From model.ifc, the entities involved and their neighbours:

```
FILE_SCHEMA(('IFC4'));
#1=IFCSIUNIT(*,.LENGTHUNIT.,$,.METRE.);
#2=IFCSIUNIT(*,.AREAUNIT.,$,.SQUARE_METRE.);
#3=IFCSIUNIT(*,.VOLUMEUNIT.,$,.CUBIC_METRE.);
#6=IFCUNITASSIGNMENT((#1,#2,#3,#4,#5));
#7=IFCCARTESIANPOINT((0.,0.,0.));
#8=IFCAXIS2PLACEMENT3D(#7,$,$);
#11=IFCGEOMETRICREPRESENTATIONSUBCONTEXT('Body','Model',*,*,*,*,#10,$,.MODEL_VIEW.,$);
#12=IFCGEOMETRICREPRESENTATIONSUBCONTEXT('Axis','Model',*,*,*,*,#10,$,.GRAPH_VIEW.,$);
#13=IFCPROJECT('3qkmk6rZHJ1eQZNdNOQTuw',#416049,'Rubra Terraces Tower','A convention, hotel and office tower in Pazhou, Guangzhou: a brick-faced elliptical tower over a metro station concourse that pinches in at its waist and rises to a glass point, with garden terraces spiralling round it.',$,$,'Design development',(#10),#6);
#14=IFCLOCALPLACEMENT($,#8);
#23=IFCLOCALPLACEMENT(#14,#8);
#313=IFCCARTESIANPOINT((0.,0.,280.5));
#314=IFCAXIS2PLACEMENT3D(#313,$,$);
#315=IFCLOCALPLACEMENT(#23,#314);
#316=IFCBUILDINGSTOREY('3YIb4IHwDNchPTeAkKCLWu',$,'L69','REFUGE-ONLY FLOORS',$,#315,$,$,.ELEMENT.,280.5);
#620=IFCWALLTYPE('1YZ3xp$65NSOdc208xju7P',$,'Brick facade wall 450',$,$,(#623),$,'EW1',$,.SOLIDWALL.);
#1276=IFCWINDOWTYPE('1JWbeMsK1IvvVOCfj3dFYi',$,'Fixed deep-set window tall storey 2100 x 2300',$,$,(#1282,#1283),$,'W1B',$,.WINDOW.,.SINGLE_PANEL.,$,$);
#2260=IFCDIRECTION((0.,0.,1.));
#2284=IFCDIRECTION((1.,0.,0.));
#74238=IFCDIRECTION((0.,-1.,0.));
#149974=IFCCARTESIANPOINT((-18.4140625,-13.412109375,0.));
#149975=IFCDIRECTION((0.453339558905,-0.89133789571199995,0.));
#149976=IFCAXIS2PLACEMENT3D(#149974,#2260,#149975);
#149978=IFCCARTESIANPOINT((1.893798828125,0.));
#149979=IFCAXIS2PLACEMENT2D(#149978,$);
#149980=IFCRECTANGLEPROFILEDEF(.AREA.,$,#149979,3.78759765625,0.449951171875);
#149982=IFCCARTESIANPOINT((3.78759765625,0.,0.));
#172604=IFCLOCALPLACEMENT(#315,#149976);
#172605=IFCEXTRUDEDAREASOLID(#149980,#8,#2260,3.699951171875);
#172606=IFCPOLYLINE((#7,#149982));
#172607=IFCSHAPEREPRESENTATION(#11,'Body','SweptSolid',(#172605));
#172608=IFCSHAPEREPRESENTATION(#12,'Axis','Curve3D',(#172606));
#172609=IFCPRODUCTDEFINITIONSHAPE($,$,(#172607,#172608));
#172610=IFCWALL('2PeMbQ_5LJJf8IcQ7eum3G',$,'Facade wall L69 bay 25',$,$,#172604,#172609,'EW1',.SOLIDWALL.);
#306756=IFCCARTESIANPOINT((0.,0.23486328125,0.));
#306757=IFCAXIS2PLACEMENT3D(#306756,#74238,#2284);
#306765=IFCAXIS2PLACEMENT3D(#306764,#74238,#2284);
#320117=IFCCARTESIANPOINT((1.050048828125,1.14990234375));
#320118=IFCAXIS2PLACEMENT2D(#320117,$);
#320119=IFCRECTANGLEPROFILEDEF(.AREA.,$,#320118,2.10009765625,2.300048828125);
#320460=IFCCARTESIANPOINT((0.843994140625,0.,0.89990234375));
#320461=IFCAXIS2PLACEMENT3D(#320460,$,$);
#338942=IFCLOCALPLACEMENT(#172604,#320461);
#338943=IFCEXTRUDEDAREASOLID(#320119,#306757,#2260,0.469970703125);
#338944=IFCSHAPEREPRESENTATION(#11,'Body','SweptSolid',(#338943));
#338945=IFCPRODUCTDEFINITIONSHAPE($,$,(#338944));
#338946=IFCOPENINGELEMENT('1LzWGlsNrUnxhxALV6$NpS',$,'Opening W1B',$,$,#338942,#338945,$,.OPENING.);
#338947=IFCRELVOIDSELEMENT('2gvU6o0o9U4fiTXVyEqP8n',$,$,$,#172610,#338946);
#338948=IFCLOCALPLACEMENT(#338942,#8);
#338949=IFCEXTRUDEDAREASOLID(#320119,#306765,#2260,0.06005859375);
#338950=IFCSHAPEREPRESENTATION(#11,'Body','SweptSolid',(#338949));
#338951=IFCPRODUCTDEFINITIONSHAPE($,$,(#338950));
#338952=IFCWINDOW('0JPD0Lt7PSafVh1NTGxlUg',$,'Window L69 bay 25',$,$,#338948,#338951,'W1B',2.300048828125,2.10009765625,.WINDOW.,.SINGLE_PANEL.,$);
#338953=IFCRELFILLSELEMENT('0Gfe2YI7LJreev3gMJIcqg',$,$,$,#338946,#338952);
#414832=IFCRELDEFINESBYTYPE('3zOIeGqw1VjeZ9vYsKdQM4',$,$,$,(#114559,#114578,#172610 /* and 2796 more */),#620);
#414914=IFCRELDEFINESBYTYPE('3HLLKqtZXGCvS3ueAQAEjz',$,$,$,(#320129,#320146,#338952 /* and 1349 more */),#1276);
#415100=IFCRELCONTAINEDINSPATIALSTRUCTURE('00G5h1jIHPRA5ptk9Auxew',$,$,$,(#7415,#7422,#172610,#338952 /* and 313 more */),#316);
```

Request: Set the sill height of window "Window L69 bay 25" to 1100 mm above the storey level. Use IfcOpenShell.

```python
import numpy as np
import ifcopenshell
import ifcopenshell.api.geometry
import ifcopenshell.geom
import ifcopenshell.util.element
import ifcopenshell.util.placement
import ifcopenshell.util.shape
import ifcopenshell.util.unit

model = ifcopenshell.open("model.ifc")
unit_scale = ifcopenshell.util.unit.calculate_unit_scale(model)

window = model.by_guid("0JPD0Lt7PSafVh1NTGxlUg")
opening = window.FillsVoids[0].RelatingOpeningElement
storey = ifcopenshell.util.element.get_container(window, ifc_class="IfcBuildingStorey")
level = ifcopenshell.util.placement.get_local_placement(storey.ObjectPlacement)[2, 3]

# The opening's origin need not be at the sill, so measure its lowest point.
shape = ifcopenshell.geom.create_shape(ifcopenshell.geom.settings(), opening)
bottom = ifcopenshell.util.shape.get_shape_bottom_elevation(shape, shape.geometry) / unit_scale
dz = level + 1.1 / unit_scale - bottom

shift = np.array([0.0, 0.0, dz])
# The window is placed relative to its opening, so it follows when the opening moves.
matrix = ifcopenshell.util.placement.get_local_placement(opening.ObjectPlacement)
matrix[:3, 3] += shift
ifcopenshell.api.geometry.edit_object_placement(
    model, product=opening, matrix=matrix, is_si=False, should_transform_children=True
)

print(f"moved by {dz * unit_scale:+.3f} m")

model.write("model_rev.ifc")
```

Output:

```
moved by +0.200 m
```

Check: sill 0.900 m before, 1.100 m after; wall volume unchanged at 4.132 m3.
